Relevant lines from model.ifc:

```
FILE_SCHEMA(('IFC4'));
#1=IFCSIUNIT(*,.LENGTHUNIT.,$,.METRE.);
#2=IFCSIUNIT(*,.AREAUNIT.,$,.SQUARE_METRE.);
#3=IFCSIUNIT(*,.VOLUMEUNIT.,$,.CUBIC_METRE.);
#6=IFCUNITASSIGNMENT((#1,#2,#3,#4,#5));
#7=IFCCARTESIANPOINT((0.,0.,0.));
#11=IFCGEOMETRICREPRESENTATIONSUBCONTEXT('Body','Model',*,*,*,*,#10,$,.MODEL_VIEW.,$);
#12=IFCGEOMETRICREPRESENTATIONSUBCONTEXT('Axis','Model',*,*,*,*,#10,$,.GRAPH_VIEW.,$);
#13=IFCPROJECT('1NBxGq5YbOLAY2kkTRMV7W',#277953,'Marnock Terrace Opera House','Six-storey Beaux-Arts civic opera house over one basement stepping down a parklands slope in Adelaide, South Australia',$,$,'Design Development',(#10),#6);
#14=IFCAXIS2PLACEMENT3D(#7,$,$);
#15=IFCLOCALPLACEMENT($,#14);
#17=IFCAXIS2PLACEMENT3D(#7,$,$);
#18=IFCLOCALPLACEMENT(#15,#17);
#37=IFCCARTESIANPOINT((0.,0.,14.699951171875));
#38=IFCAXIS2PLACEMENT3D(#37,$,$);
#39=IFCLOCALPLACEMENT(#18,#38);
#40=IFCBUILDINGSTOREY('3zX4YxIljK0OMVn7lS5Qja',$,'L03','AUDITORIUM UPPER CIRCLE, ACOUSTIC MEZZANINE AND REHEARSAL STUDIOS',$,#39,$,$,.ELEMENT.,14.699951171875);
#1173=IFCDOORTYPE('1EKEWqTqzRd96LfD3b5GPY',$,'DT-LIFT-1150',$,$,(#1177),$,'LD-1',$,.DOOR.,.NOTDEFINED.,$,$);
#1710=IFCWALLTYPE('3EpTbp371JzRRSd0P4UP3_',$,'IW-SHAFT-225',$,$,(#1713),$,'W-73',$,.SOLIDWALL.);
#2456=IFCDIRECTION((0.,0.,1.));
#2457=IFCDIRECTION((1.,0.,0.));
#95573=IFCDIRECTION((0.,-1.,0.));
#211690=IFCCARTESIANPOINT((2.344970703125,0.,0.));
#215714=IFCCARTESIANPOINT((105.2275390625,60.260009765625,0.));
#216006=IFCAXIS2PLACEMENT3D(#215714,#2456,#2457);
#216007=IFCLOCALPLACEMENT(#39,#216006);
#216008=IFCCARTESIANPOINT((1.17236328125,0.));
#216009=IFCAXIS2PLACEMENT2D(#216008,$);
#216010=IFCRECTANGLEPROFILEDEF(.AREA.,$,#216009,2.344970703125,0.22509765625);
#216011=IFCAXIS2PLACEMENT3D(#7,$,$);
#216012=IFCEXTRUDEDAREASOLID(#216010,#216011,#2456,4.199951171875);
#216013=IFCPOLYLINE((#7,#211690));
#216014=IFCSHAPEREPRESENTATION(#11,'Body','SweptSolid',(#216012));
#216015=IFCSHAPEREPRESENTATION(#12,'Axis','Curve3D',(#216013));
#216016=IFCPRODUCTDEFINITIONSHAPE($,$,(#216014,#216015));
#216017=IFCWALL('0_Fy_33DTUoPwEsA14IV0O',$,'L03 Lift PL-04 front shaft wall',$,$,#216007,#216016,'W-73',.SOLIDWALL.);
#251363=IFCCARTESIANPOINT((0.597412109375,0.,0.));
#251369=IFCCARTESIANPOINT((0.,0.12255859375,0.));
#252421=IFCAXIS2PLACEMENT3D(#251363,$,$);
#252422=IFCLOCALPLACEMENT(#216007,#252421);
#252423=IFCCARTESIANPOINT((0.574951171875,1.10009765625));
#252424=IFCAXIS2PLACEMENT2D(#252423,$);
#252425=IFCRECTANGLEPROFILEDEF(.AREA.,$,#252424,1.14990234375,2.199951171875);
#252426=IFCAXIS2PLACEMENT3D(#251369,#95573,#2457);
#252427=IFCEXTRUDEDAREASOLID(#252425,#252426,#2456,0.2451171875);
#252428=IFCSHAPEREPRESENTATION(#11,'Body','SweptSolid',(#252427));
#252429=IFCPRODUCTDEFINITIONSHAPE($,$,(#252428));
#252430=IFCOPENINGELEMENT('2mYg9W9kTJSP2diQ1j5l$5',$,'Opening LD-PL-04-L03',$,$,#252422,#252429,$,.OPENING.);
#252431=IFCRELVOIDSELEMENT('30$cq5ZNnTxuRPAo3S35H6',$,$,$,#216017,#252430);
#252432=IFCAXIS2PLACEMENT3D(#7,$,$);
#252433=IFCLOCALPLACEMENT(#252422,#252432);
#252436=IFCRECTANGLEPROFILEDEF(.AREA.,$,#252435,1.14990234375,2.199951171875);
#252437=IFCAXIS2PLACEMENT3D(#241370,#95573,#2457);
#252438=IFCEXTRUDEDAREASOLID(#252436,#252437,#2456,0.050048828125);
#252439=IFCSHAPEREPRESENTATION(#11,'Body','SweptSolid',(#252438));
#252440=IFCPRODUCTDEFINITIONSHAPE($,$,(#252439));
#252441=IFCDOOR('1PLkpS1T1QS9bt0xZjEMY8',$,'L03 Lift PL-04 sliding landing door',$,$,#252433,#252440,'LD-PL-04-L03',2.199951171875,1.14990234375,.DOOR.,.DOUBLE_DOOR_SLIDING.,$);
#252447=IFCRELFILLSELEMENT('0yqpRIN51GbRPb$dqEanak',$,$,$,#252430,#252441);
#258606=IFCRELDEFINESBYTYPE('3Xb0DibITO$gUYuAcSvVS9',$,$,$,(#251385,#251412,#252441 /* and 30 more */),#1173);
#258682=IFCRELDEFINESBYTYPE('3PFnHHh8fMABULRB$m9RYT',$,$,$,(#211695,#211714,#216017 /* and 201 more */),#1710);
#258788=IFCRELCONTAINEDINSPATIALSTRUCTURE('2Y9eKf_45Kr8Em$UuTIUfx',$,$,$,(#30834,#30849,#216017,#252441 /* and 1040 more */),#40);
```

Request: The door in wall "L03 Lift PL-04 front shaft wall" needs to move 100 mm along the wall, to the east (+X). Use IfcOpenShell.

```python
import ifcopenshell
import ifcopenshell.api.geometry
import ifcopenshell.util.placement
import ifcopenshell.util.unit

model = ifcopenshell.open("model.ifc")
unit_scale = ifcopenshell.util.unit.calculate_unit_scale(model)

door = model.by_id(252441)
opening = door.FillsVoids[0].RelatingOpeningElement
wall = opening.VoidsElements[0].RelatingBuildingElement

wall_matrix = ifcopenshell.util.placement.get_local_placement(wall.ObjectPlacement)
shift = wall_matrix[:3, 0] * 0.1 / unit_scale
before = ifcopenshell.util.placement.get_local_placement(door.ObjectPlacement)[:3, 3].copy()

# The door is placed relative to its opening, so it follows when the opening moves.
matrix = ifcopenshell.util.placement.get_local_placement(opening.ObjectPlacement)
matrix[:3, 3] += shift
ifcopenshell.api.geometry.edit_object_placement(
    model, product=opening, matrix=matrix, is_si=False, should_transform_children=True
)

after = ifcopenshell.util.placement.get_local_placement(door.ObjectPlacement)[:3, 3]
print("door moved by", (after - before).round(3) + 0.0)

model.write("model_updated.ifc")
```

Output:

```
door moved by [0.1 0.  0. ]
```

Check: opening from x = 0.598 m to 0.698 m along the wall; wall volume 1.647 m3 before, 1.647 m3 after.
